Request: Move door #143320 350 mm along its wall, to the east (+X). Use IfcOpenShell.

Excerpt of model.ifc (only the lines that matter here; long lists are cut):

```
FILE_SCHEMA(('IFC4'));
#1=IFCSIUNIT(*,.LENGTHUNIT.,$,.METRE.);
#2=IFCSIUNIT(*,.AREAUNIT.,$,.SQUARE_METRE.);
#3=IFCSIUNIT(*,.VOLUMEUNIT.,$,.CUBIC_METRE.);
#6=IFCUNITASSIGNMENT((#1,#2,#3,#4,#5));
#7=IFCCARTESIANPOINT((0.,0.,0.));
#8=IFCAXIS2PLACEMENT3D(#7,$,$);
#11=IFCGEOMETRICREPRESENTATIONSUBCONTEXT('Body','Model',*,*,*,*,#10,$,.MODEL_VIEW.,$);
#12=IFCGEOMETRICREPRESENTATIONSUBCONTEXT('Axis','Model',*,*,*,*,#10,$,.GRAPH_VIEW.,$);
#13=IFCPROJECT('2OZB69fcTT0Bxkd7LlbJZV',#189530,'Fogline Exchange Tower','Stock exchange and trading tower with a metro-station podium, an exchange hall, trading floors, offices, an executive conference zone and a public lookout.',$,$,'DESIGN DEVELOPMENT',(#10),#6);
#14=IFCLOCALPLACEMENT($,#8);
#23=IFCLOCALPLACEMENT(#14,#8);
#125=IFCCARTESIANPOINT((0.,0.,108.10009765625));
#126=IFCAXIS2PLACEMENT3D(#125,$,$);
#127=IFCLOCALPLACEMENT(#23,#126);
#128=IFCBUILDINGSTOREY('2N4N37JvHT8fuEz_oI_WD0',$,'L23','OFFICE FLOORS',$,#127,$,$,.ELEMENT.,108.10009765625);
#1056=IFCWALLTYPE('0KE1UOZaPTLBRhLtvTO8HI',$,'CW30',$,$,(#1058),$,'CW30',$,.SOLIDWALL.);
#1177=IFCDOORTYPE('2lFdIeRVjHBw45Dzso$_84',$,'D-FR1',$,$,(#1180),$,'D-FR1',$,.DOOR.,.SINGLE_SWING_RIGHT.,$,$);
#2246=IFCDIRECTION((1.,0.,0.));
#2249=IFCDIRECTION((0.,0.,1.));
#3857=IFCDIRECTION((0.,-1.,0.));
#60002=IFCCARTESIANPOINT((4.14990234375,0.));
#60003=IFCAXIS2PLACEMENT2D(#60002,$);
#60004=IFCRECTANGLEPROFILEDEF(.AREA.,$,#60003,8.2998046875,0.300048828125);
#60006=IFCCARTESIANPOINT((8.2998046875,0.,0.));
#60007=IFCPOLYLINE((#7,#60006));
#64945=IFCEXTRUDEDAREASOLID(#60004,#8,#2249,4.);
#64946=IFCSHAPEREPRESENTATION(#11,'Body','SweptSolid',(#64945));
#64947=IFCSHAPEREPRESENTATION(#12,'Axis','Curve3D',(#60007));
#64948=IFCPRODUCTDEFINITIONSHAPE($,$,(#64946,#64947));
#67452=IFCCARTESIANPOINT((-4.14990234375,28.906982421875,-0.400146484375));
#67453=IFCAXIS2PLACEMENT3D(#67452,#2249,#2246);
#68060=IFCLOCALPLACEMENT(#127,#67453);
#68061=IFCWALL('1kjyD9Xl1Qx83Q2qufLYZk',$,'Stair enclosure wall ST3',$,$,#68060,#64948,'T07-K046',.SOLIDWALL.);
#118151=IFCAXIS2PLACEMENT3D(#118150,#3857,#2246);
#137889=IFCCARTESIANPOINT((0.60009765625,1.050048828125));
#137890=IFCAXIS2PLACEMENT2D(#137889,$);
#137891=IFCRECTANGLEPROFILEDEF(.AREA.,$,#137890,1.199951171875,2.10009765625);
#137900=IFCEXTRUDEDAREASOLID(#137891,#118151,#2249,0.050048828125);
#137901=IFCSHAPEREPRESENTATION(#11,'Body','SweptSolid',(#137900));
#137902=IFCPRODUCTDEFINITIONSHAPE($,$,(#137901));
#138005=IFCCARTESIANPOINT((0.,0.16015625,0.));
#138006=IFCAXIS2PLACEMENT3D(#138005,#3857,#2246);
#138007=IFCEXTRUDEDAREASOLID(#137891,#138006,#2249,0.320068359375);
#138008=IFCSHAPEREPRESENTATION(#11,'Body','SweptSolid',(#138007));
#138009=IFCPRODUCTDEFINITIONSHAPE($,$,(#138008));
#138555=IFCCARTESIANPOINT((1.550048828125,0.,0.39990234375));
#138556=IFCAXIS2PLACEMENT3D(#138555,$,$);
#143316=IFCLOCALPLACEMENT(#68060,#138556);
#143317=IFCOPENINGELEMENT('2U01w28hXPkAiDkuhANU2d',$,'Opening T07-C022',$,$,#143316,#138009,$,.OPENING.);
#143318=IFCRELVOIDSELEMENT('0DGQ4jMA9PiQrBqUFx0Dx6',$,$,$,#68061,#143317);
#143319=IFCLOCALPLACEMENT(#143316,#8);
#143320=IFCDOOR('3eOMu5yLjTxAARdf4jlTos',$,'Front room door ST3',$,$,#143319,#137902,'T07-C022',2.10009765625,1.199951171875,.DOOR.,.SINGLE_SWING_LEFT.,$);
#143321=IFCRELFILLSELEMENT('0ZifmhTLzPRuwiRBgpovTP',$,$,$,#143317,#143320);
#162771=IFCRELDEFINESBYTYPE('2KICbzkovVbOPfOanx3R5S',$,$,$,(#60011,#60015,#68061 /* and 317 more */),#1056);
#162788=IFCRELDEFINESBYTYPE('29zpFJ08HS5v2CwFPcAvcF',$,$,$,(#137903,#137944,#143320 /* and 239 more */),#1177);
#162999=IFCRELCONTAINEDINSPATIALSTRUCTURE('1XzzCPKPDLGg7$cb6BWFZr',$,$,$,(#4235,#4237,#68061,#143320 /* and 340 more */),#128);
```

```python
import ifcopenshell
import ifcopenshell.api.geometry
import ifcopenshell.util.placement
import ifcopenshell.util.unit

model = ifcopenshell.open("model.ifc")
unit_scale = ifcopenshell.util.unit.calculate_unit_scale(model)

door = model.by_guid("3eOMu5yLjTxAARdf4jlTos")
opening = door.FillsVoids[0].RelatingOpeningElement
wall = opening.VoidsElements[0].RelatingBuildingElement

wall_matrix = ifcopenshell.util.placement.get_local_placement(wall.ObjectPlacement)
shift = wall_matrix[:3, 0] * 0.35 / unit_scale
before = ifcopenshell.util.placement.get_local_placement(door.ObjectPlacement)[:3, 3].copy()

# The door is placed relative to its opening, so it follows when the opening moves.
matrix = ifcopenshell.util.placement.get_local_placement(opening.ObjectPlacement)
matrix[:3, 3] += shift
ifcopenshell.api.geometry.edit_object_placement(
    model, product=opening, matrix=matrix, is_si=False, should_transform_children=True
)

after = ifcopenshell.util.placement.get_local_placement(door.ObjectPlacement)[:3, 3]
print("door moved by", (after - before).round(3) + 0.0)

model.write("model_edited.ifc")
```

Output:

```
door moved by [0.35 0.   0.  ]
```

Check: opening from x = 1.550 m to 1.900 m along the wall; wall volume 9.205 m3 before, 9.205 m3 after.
